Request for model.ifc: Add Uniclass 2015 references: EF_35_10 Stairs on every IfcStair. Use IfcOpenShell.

First a look at what the model holds.

```python
import ifcopenshell

model = ifcopenshell.open("model.ifc")
print(model.schema)
print("classifications:", [c.Name for c in model.by_type("IfcClassification")])
for ifc_class in ("IfcDoor", "IfcRoof", "IfcStair", "IfcWall", "IfcWindow"):
    print(ifc_class, len(model.by_type(ifc_class)))
```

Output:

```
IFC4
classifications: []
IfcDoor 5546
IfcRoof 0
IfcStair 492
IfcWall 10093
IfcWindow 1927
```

```python
import ifcopenshell
import ifcopenshell.api.classification

model = ifcopenshell.open("model.ifc")

system = ifcopenshell.api.classification.add_classification(model, classification="Uniclass 2015")

codes = {
    "IfcStair": ("EF_35_10", "Stairs"),
}
for ifc_class, (code, name) in codes.items():
    products = model.by_type(ifc_class)
    ifcopenshell.api.classification.add_reference(
        model, products=products, classification=system, identification=code, name=name
    )
    print(code, len(products))

model.write("model_v2.ifc")
```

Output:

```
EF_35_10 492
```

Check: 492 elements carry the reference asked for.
